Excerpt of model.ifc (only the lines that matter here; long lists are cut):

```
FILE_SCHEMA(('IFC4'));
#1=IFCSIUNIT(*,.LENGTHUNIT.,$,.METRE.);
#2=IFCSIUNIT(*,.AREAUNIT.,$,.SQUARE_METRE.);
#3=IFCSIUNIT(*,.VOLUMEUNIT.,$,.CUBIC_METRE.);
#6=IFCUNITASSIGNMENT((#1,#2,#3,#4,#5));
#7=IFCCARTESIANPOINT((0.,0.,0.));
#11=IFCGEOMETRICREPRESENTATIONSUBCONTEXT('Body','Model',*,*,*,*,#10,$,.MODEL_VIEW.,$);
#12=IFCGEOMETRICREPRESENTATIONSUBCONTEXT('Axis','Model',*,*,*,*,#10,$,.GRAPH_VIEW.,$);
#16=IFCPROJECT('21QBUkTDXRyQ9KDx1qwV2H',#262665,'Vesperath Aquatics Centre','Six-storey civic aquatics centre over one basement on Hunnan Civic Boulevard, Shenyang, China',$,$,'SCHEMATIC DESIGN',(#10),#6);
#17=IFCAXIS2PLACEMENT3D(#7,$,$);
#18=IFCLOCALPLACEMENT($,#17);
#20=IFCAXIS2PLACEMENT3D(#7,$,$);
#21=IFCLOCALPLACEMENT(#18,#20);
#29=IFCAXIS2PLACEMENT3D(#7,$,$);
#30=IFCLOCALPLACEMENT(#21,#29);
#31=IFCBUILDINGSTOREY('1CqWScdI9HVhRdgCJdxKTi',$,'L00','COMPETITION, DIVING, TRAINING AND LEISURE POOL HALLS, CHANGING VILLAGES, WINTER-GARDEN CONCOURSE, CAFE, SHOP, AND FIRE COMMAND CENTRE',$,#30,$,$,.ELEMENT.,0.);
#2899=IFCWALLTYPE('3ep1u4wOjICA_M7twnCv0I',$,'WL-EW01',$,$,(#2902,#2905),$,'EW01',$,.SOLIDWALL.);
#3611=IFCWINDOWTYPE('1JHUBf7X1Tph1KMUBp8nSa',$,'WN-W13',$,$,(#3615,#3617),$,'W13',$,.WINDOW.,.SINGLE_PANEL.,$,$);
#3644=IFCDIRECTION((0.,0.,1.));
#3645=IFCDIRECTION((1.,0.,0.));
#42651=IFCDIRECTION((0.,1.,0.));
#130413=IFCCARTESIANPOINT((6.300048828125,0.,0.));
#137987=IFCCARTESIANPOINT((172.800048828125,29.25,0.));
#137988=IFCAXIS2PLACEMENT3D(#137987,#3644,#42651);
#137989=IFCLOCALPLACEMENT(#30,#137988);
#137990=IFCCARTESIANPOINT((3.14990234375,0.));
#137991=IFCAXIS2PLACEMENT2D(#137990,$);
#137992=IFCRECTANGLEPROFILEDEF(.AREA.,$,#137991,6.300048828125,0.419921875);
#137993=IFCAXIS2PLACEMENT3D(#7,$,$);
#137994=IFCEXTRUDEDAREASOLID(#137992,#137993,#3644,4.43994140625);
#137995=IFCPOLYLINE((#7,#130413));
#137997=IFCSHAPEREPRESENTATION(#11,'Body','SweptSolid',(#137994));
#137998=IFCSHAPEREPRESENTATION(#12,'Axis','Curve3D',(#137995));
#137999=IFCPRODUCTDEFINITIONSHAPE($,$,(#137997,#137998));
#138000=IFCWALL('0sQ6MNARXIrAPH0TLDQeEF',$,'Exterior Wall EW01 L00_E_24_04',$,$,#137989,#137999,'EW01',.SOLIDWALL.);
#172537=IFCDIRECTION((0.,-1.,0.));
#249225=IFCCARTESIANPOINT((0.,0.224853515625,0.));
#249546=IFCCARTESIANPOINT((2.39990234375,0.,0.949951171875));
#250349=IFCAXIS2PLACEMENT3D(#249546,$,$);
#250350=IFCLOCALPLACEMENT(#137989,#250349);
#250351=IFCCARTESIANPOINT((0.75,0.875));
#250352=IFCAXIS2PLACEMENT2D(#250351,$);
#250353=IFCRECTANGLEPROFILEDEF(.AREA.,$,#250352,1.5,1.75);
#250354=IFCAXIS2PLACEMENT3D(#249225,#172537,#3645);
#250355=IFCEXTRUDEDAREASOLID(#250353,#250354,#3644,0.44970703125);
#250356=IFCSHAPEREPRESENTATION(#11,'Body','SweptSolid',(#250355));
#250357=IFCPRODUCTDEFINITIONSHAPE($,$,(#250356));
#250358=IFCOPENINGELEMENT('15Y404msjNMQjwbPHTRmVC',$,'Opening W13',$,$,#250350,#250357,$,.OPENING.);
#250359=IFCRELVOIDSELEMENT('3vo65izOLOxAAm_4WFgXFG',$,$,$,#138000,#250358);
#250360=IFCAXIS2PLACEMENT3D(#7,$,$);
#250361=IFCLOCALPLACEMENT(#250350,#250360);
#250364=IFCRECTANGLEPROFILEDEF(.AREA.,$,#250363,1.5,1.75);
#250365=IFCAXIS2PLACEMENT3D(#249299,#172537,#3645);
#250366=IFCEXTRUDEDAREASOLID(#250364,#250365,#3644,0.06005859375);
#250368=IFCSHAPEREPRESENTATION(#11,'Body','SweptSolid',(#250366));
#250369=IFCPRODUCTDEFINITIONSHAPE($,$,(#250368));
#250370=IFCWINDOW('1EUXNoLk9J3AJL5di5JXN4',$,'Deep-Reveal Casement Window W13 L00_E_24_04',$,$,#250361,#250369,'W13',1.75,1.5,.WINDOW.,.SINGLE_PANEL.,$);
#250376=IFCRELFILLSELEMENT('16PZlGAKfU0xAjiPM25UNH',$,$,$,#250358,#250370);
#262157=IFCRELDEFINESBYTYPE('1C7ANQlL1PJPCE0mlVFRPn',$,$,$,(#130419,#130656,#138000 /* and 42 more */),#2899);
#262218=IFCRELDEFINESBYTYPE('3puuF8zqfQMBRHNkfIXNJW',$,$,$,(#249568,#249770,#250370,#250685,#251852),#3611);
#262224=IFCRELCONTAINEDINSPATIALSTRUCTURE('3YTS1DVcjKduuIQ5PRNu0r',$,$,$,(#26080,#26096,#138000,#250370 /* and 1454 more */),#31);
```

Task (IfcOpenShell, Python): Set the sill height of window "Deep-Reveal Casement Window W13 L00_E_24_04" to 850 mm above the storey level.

```python
import numpy as np
import ifcopenshell
import ifcopenshell.api.geometry
import ifcopenshell.geom
import ifcopenshell.util.element
import ifcopenshell.util.placement
import ifcopenshell.util.shape
import ifcopenshell.util.unit

model = ifcopenshell.open("model.ifc")
unit_scale = ifcopenshell.util.unit.calculate_unit_scale(model)

window = model.by_guid("1EUXNoLk9J3AJL5di5JXN4")
opening = window.FillsVoids[0].RelatingOpeningElement
storey = ifcopenshell.util.element.get_container(window, ifc_class="IfcBuildingStorey")
level = ifcopenshell.util.placement.get_local_placement(storey.ObjectPlacement)[2, 3]

# The opening's origin need not be at the sill, so measure its lowest point.
shape = ifcopenshell.geom.create_shape(ifcopenshell.geom.settings(), opening)
bottom = ifcopenshell.util.shape.get_shape_bottom_elevation(shape, shape.geometry) / unit_scale
dz = level + 0.85 - bottom

shift = np.array([0.0, 0.0, dz])
# The window is placed relative to its opening, so it follows when the opening moves.
matrix = ifcopenshell.util.placement.get_local_placement(opening.ObjectPlacement)
matrix[:3, 3] += shift
ifcopenshell.api.geometry.edit_object_placement(
    model, product=opening, matrix=matrix, is_si=False, should_transform_children=True
)

print(f"moved by {dz * unit_scale:+.3f} m")

model.write("model_edited.ifc")
```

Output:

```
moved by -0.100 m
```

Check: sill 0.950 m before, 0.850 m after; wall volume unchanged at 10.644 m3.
